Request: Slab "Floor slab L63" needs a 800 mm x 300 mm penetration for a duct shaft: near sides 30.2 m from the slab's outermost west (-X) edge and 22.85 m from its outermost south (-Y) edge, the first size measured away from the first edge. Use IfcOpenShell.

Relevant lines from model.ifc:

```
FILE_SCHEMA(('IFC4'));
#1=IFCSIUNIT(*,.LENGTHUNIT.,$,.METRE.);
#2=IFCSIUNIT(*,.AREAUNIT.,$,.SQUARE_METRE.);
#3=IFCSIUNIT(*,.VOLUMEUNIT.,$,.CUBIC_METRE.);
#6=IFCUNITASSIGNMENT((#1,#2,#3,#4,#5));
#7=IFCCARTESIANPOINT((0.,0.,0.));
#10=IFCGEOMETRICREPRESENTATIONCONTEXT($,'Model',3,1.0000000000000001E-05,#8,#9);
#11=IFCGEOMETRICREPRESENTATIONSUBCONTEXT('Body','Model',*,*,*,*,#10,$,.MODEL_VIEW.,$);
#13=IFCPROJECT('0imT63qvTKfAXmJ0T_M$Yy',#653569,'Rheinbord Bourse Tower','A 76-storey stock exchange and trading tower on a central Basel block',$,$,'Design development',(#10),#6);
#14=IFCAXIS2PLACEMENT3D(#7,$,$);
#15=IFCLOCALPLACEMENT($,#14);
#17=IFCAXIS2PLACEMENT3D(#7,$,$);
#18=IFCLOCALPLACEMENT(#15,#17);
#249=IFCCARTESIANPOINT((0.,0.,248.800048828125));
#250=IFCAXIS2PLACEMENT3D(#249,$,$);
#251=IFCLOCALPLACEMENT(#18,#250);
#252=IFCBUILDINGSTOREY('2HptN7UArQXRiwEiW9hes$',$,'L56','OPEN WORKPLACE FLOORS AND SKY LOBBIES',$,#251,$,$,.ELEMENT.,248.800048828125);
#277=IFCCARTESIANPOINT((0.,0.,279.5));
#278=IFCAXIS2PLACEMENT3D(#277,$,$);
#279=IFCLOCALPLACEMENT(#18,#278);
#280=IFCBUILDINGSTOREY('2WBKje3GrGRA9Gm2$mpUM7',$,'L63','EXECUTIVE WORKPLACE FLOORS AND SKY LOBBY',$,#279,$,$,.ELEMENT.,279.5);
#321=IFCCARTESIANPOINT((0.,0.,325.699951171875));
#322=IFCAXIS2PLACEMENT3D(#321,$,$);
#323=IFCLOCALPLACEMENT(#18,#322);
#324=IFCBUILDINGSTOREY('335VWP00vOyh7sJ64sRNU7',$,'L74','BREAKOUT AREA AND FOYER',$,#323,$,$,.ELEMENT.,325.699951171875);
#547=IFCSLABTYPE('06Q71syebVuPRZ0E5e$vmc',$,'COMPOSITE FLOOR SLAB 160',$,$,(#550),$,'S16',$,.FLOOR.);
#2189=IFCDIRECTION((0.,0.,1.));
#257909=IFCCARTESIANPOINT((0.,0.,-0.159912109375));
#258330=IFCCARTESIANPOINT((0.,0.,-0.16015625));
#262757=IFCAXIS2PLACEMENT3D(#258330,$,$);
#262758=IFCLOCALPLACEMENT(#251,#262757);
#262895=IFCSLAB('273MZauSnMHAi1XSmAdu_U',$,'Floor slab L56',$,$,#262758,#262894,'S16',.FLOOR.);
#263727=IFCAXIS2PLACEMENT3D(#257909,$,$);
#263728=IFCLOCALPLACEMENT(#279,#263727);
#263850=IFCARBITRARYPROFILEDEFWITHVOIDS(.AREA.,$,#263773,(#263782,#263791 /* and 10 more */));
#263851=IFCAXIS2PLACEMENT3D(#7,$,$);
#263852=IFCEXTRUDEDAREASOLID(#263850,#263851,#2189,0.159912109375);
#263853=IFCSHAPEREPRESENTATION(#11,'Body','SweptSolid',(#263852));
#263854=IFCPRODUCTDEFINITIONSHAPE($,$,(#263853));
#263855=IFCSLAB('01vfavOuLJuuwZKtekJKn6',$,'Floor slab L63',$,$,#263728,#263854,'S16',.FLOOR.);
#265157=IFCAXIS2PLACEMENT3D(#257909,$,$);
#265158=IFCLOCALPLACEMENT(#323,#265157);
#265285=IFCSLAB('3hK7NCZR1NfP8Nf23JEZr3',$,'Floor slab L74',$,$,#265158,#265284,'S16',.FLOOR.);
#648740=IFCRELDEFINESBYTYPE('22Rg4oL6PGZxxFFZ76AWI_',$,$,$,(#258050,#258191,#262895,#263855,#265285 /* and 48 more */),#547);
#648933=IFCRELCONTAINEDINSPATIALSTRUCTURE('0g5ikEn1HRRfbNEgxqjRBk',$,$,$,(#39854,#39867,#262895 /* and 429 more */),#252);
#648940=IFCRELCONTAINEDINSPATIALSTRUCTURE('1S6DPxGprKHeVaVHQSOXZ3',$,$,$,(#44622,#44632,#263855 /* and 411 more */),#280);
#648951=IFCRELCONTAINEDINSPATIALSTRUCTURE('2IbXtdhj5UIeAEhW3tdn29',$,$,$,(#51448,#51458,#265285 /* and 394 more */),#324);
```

```python
import numpy as np
import ifcopenshell
import ifcopenshell.api.feature
import ifcopenshell.api.geometry
import ifcopenshell.api.root
import ifcopenshell.geom
import ifcopenshell.util.placement
import ifcopenshell.util.representation
import ifcopenshell.util.shape
import ifcopenshell.util.unit

model = ifcopenshell.open("model.ifc")
unit_scale = ifcopenshell.util.unit.calculate_unit_scale(model)
settings = ifcopenshell.geom.settings()


def volume(element):
    """Net volume in cubic metres, openings subtracted."""
    shape = ifcopenshell.geom.create_shape(settings, element)
    return ifcopenshell.util.shape.get_volume(shape.geometry)


slab = model.by_id(263855)
before = volume(slab)

# Extent in the slab's own axes, in metres. The edges named are its -X and -Y sides.
slab_shape = ifcopenshell.geom.create_shape(settings, slab)
vertices = ifcopenshell.util.shape.get_vertices(slab_shape.geometry)
x_min, y_min, bottom = vertices.min(axis=0)
top = vertices[:, 2].max()

opening = ifcopenshell.api.root.create_entity(model, ifc_class="IfcOpeningElement", name="Duct shaft opening", predefined_type="OPENING")
context = ifcopenshell.util.representation.get_context(model, "Model", "Body", "MODEL_VIEW")
width, depth = 0.8, 0.3
outline = [(0.0, 0.0), (width, 0.0), (width, depth), (0.0, depth), (0.0, 0.0)]
# Overshoot both faces by 50 mm so the cut is clean.
shape = ifcopenshell.api.geometry.add_slab_representation(
    model, context=context, depth=top - bottom + 0.1, polyline=outline
)
ifcopenshell.api.geometry.assign_representation(model, product=opening, representation=shape)

matrix = ifcopenshell.util.placement.get_local_placement(slab.ObjectPlacement)
matrix[:, 3] = matrix @ np.append(np.array([x_min + 30.2, y_min + 22.85, bottom - 0.05]) / unit_scale, 1.0)
ifcopenshell.api.geometry.edit_object_placement(model, product=opening, matrix=matrix, is_si=False)
ifcopenshell.api.feature.add_feature(model, feature=opening, element=slab)

after = volume(slab)

print(f"slab volume {before:.3f} -> {after:.3f} m3")

model.write("model_rev.ifc")
```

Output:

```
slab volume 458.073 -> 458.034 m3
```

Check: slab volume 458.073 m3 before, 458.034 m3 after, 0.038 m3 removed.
